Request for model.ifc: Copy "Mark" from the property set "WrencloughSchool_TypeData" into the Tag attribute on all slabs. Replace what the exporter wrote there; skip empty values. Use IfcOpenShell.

First a look at what the model holds.

```python
import ifcopenshell
import ifcopenshell.util.element

model = ifcopenshell.open("model.ifc")
print(model.schema)
slabs = model.by_type("IfcSlab")
print(len(slabs), "slabs")
for e in slabs[:8]:
    source = ifcopenshell.util.element.get_pset(e, "WrencloughSchool_TypeData", "Mark")
    target = e.Tag
    print(e.id(), repr(source), repr(target), sep=" | ")
```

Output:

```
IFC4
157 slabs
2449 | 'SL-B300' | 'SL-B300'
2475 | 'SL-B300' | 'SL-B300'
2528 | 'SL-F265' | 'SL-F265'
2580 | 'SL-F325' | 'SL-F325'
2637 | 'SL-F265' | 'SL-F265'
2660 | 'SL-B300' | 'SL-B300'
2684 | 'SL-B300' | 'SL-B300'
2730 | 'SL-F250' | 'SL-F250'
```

```python
import ifcopenshell
import ifcopenshell.util.element

model = ifcopenshell.open("model.ifc")

count = 0
for e in model.by_type("IfcSlab"):
    value = ifcopenshell.util.element.get_pset(e, "WrencloughSchool_TypeData", "Mark")
    current = e.Tag
    if not value or not value.strip() or current == value:
        continue
    e.Tag = value
    count += 1

print(count, "slabs updated")

model.write("model_updated.ifc")
```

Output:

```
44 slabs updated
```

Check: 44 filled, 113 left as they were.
